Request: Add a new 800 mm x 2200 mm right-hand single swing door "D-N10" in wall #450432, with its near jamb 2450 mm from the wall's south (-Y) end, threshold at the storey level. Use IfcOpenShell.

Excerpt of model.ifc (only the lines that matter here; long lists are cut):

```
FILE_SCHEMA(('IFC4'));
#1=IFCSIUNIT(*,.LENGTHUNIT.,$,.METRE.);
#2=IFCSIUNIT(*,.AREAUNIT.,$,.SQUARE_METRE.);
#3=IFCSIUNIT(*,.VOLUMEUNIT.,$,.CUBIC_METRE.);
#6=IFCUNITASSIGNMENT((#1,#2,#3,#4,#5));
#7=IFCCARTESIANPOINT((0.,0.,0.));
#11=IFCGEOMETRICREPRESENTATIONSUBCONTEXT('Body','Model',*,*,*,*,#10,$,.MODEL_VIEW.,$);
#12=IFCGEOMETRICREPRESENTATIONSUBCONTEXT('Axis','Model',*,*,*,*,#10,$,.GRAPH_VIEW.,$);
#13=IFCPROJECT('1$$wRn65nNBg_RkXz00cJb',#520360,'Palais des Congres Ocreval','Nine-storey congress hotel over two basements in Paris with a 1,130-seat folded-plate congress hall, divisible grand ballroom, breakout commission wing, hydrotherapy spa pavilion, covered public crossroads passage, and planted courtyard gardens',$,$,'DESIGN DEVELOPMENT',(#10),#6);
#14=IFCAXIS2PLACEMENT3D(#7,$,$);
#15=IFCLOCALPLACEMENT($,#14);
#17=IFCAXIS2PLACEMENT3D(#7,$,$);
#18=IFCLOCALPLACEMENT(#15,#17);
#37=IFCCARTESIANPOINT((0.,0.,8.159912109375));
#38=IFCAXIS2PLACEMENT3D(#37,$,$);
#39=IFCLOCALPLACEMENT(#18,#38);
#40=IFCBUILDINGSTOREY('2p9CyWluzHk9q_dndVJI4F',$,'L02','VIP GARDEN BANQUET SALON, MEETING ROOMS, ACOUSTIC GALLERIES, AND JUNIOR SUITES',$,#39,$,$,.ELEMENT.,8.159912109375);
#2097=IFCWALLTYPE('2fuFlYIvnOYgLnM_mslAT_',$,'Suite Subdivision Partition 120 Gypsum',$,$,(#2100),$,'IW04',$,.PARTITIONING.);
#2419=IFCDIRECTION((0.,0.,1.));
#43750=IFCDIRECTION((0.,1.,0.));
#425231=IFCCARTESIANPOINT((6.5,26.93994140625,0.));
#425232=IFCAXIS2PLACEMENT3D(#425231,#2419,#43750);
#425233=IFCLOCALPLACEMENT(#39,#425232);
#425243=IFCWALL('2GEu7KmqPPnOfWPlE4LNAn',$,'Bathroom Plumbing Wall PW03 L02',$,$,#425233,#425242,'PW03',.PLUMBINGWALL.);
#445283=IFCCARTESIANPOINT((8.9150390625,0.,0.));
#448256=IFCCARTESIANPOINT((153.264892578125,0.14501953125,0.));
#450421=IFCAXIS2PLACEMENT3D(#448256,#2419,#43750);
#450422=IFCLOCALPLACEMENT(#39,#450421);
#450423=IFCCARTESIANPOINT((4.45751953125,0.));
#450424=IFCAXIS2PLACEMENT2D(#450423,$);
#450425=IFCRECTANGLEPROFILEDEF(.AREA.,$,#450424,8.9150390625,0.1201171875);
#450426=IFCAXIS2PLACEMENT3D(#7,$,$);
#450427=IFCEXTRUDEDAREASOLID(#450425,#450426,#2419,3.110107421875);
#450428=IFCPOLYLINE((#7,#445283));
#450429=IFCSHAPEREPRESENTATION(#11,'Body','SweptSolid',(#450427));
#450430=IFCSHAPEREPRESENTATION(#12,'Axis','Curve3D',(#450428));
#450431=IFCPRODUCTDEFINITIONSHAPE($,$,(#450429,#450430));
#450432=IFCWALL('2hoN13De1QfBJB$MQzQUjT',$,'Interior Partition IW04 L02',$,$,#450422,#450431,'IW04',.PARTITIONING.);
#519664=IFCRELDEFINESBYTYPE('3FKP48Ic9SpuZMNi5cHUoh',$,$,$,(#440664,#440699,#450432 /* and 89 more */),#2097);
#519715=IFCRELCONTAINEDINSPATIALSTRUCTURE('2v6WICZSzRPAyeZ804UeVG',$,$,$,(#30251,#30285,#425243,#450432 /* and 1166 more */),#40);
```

```python
import numpy as np
import ifcopenshell
import ifcopenshell.api.feature
import ifcopenshell.api.geometry
import ifcopenshell.api.root
import ifcopenshell.api.spatial
import ifcopenshell.geom
import ifcopenshell.util.element
import ifcopenshell.util.placement
import ifcopenshell.util.representation
import ifcopenshell.util.shape
import ifcopenshell.util.unit

model = ifcopenshell.open("model.ifc")
unit_scale = ifcopenshell.util.unit.calculate_unit_scale(model)
settings = ifcopenshell.geom.settings()


def volume(element):
    """Net volume in cubic metres, openings subtracted."""
    shape = ifcopenshell.geom.create_shape(settings, element)
    return ifcopenshell.util.shape.get_volume(shape.geometry)


wall = model.by_id(450432)
storey = ifcopenshell.util.element.get_container(wall, ifc_class="IfcBuildingStorey")
context = ifcopenshell.util.representation.get_context(model, "Model", "Body", "MODEL_VIEW")
before = volume(wall)

width, height, from_end, sill = 0.8, 2.2, 2.45, 0.0  # metres

# The wall runs along its own X axis, and the end named is its -X end.
wall_shape = ifcopenshell.geom.create_shape(settings, wall)
x, y, z = ifcopenshell.util.shape.get_vertices(wall_shape.geometry).T
start = x.min() + from_end
face, thickness = float(y.min()), float(y.max() - y.min())
wall_matrix = ifcopenshell.util.placement.get_local_placement(wall.ObjectPlacement)
level = ifcopenshell.util.placement.get_local_placement(storey.ObjectPlacement)[2, 3]


def in_wall(x, y):
    """Placement at x, y metres in the wall's axes, at sill height."""
    matrix = wall_matrix.copy()
    matrix[:, 3] = wall_matrix @ np.array([x / unit_scale, y / unit_scale, 0.0, 1.0])
    matrix[2, 3] = level + sill / unit_scale
    return matrix


# Opening: a box that overshoots both wall faces by 50 mm.
opening = ifcopenshell.api.root.create_entity(model, ifc_class="IfcOpeningElement", predefined_type="OPENING")
box = ifcopenshell.api.geometry.add_wall_representation(
    model, context=context, length=width, height=height, thickness=thickness + 0.1
)
ifcopenshell.api.geometry.assign_representation(model, product=opening, representation=box)
ifcopenshell.api.geometry.edit_object_placement(model, product=opening, matrix=in_wall(start, face - 0.05), is_si=False)
ifcopenshell.api.feature.add_feature(model, feature=opening, element=wall)

door = ifcopenshell.api.root.create_entity(model, ifc_class="IfcDoor", name="D-N10", predefined_type="DOOR")
door.OverallWidth, door.OverallHeight = width / unit_scale, height / unit_scale
door.OperationType = "SINGLE_SWING_RIGHT"
body = ifcopenshell.api.geometry.add_door_representation(
    model,
    context=context,
    overall_width=door.OverallWidth,
    overall_height=door.OverallHeight,
    operation_type="SINGLE_SWING_RIGHT",
    lining_properties={"LiningDepth": thickness / unit_scale, "ThresholdDepth": thickness / unit_scale},
)
ifcopenshell.api.geometry.assign_representation(model, product=door, representation=body)
ifcopenshell.api.spatial.assign_container(model, products=[door], relating_structure=storey)
ifcopenshell.api.feature.add_filling(model, opening=opening, element=door)

# The lining spans the wall, so the door starts at the wall face.
ifcopenshell.api.geometry.edit_object_placement(model, product=door, matrix=in_wall(start, face), is_si=False)

after = volume(wall)

print(f"wall volume {before:.3f} -> {after:.3f} m3")

model.write("model_updated.ifc")
```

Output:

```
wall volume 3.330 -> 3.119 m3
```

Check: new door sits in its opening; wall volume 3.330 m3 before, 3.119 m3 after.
